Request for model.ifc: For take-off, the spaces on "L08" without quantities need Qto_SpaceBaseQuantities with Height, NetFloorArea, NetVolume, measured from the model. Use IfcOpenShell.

First a look at what the model holds.

```python
import ifcopenshell
import ifcopenshell.util.element
import ifcopenshell.util.unit

model = ifcopenshell.open("model.ifc")
print(model.schema)
for unit_type in ("LENGTHUNIT", "AREAUNIT", "VOLUMEUNIT"):
    print(unit_type, ifcopenshell.util.unit.calculate_unit_scale(model, unit_type))
storey = next(s for s in model.by_type("IfcBuildingStorey") if s.Name == "L08")
spaces = [e for e in ifcopenshell.util.element.get_decomposition(storey) if e.is_a("IfcSpace")]
for e in sorted(spaces, key=lambda e: e.id()):
    print(e.id(), e.is_a(), e.Name, list(ifcopenshell.util.element.get_psets(e, qtos_only=True)), sep=" | ")
```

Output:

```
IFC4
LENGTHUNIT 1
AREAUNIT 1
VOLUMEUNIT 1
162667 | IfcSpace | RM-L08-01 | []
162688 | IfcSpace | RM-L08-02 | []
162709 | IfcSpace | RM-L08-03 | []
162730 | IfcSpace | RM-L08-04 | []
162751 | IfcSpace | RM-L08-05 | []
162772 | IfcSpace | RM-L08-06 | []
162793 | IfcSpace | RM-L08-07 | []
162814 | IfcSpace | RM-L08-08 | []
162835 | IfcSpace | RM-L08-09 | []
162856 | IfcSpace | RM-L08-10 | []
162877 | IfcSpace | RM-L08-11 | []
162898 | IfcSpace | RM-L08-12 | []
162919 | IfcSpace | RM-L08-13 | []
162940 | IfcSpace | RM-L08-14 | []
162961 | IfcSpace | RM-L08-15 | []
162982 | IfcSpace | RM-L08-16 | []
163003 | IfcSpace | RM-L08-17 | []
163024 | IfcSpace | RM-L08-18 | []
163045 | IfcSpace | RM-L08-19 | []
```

```python
import ifcopenshell
import ifcopenshell.api.pset
import ifcopenshell.geom
import ifcopenshell.util.element
import ifcopenshell.util.shape
import ifcopenshell.util.unit

model = ifcopenshell.open("model.ifc")
unit_scale = ifcopenshell.util.unit.calculate_unit_scale(model)
area_scale = ifcopenshell.util.unit.calculate_unit_scale(model, "AREAUNIT")
volume_scale = ifcopenshell.util.unit.calculate_unit_scale(model, "VOLUMEUNIT")
settings = ifcopenshell.geom.settings()

storey = next(s for s in model.by_type("IfcBuildingStorey") if s.Name == "L08")
spaces = [e for e in ifcopenshell.util.element.get_decomposition(storey) if e.is_a("IfcSpace")]

for e in sorted(spaces, key=lambda e: e.id()):
    if ifcopenshell.util.element.get_psets(e, qtos_only=True, should_inherit=False):
        continue
    # Geometry comes back in metres, in the element's own axes.
    shape = ifcopenshell.geom.create_shape(settings, e)
    values = {
        "Height": ifcopenshell.util.shape.get_z(shape.geometry) / unit_scale,
        "NetFloorArea": ifcopenshell.util.shape.get_footprint_area(shape.geometry) / area_scale,
        "NetVolume": ifcopenshell.util.shape.get_volume(shape.geometry) / volume_scale,
    }
    qto = ifcopenshell.api.pset.add_qto(model, product=e, name="Qto_SpaceBaseQuantities")
    ifcopenshell.api.pset.edit_qto(model, qto=qto, properties=values)
    print(e.id(), {k: round(v, 3) for k, v in values.items()})

model.write("model_v2.ifc")
```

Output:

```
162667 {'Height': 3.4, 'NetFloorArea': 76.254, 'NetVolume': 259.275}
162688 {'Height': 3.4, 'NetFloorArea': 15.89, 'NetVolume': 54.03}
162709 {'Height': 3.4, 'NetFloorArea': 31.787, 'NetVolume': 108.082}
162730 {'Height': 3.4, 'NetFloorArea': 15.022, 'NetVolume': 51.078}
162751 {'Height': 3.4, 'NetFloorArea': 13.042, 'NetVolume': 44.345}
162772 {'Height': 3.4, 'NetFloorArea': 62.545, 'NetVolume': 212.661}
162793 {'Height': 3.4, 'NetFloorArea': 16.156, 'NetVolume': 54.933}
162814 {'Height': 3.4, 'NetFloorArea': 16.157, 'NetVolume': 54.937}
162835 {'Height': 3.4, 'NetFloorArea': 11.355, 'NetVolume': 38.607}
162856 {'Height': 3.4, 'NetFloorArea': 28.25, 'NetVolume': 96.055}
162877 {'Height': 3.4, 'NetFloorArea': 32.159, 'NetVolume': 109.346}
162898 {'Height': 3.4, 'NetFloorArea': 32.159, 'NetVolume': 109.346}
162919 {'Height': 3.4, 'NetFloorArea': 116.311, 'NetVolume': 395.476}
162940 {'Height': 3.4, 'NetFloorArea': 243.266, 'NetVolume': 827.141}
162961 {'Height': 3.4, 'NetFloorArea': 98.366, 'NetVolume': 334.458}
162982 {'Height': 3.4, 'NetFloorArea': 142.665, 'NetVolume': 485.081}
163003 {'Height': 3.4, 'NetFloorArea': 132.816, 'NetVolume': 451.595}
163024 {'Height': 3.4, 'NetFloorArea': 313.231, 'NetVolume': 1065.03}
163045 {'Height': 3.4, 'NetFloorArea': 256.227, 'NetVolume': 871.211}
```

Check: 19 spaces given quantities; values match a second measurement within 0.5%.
